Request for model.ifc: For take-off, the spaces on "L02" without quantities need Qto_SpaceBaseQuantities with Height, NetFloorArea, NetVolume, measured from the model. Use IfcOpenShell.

First a look at what the model holds.

```python
import ifcopenshell
import ifcopenshell.util.element
import ifcopenshell.util.unit

model = ifcopenshell.open("model.ifc")
print(model.schema)
for unit_type in ("LENGTHUNIT", "AREAUNIT", "VOLUMEUNIT"):
    print(unit_type, ifcopenshell.util.unit.calculate_unit_scale(model, unit_type))
storey = next(s for s in model.by_type("IfcBuildingStorey") if s.Name == "L02")
spaces = [e for e in ifcopenshell.util.element.get_decomposition(storey) if e.is_a("IfcSpace")]
for e in sorted(spaces, key=lambda e: e.id()):
    print(e.id(), e.is_a(), e.Name, list(ifcopenshell.util.element.get_psets(e, qtos_only=True)), sep=" | ")
```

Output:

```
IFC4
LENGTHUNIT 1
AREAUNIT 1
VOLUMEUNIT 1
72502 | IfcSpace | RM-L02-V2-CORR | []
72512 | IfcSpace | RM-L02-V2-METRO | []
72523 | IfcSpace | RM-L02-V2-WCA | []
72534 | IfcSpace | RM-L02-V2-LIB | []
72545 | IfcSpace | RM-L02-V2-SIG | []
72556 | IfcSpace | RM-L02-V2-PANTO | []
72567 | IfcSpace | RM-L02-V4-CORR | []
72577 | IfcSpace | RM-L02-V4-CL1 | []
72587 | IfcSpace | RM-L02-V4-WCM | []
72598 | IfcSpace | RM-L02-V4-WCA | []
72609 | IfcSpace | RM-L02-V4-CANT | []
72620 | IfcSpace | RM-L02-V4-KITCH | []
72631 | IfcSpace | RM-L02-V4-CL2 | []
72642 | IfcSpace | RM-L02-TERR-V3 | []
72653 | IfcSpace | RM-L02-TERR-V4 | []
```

```python
import ifcopenshell
import ifcopenshell.api.pset
import ifcopenshell.geom
import ifcopenshell.util.element
import ifcopenshell.util.shape
import ifcopenshell.util.unit

model = ifcopenshell.open("model.ifc")
unit_scale = ifcopenshell.util.unit.calculate_unit_scale(model)
area_scale = ifcopenshell.util.unit.calculate_unit_scale(model, "AREAUNIT")
volume_scale = ifcopenshell.util.unit.calculate_unit_scale(model, "VOLUMEUNIT")
settings = ifcopenshell.geom.settings()

storey = next(s for s in model.by_type("IfcBuildingStorey") if s.Name == "L02")
spaces = [e for e in ifcopenshell.util.element.get_decomposition(storey) if e.is_a("IfcSpace")]

for e in sorted(spaces, key=lambda e: e.id()):
    if ifcopenshell.util.element.get_psets(e, qtos_only=True, should_inherit=False):
        continue
    # Geometry comes back in metres, in the element's own axes.
    shape = ifcopenshell.geom.create_shape(settings, e)
    values = {
        "Height": ifcopenshell.util.shape.get_z(shape.geometry) / unit_scale,
        "NetFloorArea": ifcopenshell.util.shape.get_footprint_area(shape.geometry) / area_scale,
        "NetVolume": ifcopenshell.util.shape.get_volume(shape.geometry) / volume_scale,
    }
    qto = ifcopenshell.api.pset.add_qto(model, product=e, name="Qto_SpaceBaseQuantities")
    ifcopenshell.api.pset.edit_qto(model, qto=qto, properties=values)
    print(e.id(), {k: round(v, 3) for k, v in values.items()})

model.write("model_updated.ifc")
```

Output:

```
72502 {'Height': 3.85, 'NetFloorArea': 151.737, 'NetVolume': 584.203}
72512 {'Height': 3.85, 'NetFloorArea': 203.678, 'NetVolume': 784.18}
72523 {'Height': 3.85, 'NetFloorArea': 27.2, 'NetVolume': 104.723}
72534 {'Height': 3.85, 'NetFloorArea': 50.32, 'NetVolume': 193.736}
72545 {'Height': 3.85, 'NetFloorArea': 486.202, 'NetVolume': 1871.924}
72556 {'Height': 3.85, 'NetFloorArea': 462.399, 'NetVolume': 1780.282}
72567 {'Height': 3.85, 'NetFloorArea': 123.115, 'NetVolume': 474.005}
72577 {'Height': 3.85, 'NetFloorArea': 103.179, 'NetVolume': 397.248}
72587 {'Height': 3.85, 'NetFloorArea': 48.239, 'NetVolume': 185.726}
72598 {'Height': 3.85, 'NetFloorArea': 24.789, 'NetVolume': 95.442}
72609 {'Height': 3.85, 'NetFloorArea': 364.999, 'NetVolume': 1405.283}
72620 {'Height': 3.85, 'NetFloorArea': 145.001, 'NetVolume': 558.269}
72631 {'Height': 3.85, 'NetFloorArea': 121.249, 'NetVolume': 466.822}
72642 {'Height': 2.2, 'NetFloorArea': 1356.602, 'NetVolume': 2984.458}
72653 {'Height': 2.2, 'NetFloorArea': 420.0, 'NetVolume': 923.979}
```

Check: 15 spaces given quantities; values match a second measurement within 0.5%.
